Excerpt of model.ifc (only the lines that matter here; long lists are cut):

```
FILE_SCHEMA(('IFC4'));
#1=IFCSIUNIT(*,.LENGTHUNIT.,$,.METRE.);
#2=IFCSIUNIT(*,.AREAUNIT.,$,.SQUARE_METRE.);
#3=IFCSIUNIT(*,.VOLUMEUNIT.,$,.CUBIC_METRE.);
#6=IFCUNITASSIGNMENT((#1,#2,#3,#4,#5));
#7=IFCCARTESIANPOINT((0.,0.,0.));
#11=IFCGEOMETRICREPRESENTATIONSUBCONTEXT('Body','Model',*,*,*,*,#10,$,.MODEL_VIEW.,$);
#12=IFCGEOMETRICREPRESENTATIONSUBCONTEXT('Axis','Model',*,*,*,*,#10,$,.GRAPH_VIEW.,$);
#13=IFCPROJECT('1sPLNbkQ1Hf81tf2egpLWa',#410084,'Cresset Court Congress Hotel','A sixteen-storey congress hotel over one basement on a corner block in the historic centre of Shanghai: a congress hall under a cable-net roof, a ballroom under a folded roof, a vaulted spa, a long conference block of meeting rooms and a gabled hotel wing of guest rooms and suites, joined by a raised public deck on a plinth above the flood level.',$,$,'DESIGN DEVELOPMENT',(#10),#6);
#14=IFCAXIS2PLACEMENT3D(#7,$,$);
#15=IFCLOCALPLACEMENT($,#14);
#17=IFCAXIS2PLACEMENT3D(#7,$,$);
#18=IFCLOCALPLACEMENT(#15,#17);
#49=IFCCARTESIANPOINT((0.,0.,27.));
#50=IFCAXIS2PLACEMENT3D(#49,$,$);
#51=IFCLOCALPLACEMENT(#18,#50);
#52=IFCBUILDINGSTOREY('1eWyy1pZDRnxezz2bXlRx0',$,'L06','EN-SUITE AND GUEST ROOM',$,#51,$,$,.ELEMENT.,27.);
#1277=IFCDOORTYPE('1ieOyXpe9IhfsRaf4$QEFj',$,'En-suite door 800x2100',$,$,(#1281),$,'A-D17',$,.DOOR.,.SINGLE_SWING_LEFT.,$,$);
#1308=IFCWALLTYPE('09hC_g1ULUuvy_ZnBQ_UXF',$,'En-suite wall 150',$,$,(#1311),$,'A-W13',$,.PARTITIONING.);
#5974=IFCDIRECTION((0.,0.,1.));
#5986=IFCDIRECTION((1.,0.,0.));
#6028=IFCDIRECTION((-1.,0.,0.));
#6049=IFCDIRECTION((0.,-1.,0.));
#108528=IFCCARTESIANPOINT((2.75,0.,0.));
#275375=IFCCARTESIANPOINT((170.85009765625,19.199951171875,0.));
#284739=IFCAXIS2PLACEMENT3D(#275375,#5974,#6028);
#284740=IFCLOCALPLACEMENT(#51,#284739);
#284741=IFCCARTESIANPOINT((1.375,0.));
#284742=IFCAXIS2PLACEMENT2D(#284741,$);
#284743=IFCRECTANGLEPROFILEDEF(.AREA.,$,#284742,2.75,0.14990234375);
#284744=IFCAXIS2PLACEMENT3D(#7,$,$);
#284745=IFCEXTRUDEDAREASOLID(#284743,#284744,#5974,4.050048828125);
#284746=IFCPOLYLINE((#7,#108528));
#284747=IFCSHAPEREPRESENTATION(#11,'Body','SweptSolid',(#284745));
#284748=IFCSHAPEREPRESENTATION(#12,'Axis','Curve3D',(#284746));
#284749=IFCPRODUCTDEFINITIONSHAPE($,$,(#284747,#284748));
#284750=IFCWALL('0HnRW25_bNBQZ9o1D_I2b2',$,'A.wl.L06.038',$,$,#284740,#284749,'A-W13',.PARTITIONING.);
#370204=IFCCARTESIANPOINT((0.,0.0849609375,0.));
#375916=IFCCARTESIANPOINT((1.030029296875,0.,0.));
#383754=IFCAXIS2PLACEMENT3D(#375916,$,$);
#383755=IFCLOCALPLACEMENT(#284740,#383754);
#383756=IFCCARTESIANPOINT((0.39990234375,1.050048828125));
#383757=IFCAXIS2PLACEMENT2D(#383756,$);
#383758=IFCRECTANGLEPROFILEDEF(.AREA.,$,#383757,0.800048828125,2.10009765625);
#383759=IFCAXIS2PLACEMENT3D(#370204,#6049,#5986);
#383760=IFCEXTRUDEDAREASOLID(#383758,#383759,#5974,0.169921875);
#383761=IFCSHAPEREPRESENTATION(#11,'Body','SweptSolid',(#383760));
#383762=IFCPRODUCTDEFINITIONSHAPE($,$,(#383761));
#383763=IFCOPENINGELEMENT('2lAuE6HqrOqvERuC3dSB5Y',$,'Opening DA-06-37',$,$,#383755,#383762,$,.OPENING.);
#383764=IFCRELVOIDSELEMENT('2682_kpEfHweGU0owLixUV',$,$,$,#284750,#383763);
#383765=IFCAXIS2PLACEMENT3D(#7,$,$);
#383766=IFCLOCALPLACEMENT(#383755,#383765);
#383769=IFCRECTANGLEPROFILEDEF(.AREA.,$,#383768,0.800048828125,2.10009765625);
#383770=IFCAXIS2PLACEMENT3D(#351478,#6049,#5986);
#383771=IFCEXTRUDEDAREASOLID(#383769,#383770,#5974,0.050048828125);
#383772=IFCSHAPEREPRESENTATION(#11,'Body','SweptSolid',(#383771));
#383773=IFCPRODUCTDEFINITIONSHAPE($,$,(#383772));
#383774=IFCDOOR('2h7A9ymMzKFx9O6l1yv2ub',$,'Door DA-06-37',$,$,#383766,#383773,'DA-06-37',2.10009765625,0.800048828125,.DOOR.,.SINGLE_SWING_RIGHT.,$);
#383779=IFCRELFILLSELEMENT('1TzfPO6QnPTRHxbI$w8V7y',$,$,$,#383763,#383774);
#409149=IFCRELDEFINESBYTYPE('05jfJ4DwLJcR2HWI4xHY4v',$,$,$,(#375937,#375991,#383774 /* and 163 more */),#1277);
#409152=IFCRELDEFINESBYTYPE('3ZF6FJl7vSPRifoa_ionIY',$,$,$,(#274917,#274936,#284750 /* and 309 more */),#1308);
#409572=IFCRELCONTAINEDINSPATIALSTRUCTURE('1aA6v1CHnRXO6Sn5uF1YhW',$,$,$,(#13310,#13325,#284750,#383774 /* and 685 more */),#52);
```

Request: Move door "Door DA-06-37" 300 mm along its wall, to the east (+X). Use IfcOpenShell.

```python
import ifcopenshell
import ifcopenshell.api.geometry
import ifcopenshell.util.placement
import ifcopenshell.util.unit

model = ifcopenshell.open("model.ifc")
unit_scale = ifcopenshell.util.unit.calculate_unit_scale(model)

door = model.by_guid("2h7A9ymMzKFx9O6l1yv2ub")
opening = door.FillsVoids[0].RelatingOpeningElement
wall = opening.VoidsElements[0].RelatingBuildingElement

wall_matrix = ifcopenshell.util.placement.get_local_placement(wall.ObjectPlacement)
shift = wall_matrix[:3, 0] * -0.3 / unit_scale
before = ifcopenshell.util.placement.get_local_placement(door.ObjectPlacement)[:3, 3].copy()

# The door is placed relative to its opening, so it follows when the opening moves.
matrix = ifcopenshell.util.placement.get_local_placement(opening.ObjectPlacement)
matrix[:3, 3] += shift
ifcopenshell.api.geometry.edit_object_placement(
    model, product=opening, matrix=matrix, is_si=False, should_transform_children=True
)

after = ifcopenshell.util.placement.get_local_placement(door.ObjectPlacement)[:3, 3]
print("door moved by", (after - before).round(3) + 0.0)

model.write("model_rev.ifc")
```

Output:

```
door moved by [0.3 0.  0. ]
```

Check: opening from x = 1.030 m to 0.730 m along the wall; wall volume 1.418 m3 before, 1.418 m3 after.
